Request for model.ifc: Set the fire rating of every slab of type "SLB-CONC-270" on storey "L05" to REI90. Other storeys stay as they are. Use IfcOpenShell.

First a look at what the model holds.

```python
import ifcopenshell
import ifcopenshell.util.element

model = ifcopenshell.open("model.ifc")
print(model.schema)
storey = next(s for s in model.by_type("IfcBuildingStorey") if s.Name == "L05")
slabs = [e for e in ifcopenshell.util.element.get_decomposition(storey) if e.is_a("IfcSlab")]
seen = {}
for e in slabs:
    element_type = ifcopenshell.util.element.get_type(e)
    key = (element_type.Name if element_type != e and element_type else None, ifcopenshell.util.element.get_pset(e, "Pset_SlabCommon", "FireRating"))
    seen[key] = seen.get(key, 0) + 1
for (name, value), count in sorted(seen.items(), key=str):
    print(count, "x", name, "|", value)
```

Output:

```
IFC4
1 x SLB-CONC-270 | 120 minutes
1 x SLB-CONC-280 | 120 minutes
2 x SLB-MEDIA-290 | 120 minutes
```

```python
import ifcopenshell
import ifcopenshell.api.pset
import ifcopenshell.util.element

model = ifcopenshell.open("model.ifc")

storey = next(s for s in model.by_type("IfcBuildingStorey") if s.Name == "L05")
slabs = [e for e in ifcopenshell.util.element.get_decomposition(storey) if e.is_a("IfcSlab")]

count = 0
for e in slabs:
    element_type = ifcopenshell.util.element.get_type(e)
    if element_type in (None, e) or element_type.Name != "SLB-CONC-270":
        continue
    # add_pset returns the element's existing set when there is one.
    pset = ifcopenshell.api.pset.add_pset(model, product=e, name="Pset_SlabCommon")
    ifcopenshell.api.pset.edit_pset(model, pset=pset, properties={"FireRating": "REI90"})
    count += 1

print(count, "slabs updated")

model.write("model_rev.ifc")
```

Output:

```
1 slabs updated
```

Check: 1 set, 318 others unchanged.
